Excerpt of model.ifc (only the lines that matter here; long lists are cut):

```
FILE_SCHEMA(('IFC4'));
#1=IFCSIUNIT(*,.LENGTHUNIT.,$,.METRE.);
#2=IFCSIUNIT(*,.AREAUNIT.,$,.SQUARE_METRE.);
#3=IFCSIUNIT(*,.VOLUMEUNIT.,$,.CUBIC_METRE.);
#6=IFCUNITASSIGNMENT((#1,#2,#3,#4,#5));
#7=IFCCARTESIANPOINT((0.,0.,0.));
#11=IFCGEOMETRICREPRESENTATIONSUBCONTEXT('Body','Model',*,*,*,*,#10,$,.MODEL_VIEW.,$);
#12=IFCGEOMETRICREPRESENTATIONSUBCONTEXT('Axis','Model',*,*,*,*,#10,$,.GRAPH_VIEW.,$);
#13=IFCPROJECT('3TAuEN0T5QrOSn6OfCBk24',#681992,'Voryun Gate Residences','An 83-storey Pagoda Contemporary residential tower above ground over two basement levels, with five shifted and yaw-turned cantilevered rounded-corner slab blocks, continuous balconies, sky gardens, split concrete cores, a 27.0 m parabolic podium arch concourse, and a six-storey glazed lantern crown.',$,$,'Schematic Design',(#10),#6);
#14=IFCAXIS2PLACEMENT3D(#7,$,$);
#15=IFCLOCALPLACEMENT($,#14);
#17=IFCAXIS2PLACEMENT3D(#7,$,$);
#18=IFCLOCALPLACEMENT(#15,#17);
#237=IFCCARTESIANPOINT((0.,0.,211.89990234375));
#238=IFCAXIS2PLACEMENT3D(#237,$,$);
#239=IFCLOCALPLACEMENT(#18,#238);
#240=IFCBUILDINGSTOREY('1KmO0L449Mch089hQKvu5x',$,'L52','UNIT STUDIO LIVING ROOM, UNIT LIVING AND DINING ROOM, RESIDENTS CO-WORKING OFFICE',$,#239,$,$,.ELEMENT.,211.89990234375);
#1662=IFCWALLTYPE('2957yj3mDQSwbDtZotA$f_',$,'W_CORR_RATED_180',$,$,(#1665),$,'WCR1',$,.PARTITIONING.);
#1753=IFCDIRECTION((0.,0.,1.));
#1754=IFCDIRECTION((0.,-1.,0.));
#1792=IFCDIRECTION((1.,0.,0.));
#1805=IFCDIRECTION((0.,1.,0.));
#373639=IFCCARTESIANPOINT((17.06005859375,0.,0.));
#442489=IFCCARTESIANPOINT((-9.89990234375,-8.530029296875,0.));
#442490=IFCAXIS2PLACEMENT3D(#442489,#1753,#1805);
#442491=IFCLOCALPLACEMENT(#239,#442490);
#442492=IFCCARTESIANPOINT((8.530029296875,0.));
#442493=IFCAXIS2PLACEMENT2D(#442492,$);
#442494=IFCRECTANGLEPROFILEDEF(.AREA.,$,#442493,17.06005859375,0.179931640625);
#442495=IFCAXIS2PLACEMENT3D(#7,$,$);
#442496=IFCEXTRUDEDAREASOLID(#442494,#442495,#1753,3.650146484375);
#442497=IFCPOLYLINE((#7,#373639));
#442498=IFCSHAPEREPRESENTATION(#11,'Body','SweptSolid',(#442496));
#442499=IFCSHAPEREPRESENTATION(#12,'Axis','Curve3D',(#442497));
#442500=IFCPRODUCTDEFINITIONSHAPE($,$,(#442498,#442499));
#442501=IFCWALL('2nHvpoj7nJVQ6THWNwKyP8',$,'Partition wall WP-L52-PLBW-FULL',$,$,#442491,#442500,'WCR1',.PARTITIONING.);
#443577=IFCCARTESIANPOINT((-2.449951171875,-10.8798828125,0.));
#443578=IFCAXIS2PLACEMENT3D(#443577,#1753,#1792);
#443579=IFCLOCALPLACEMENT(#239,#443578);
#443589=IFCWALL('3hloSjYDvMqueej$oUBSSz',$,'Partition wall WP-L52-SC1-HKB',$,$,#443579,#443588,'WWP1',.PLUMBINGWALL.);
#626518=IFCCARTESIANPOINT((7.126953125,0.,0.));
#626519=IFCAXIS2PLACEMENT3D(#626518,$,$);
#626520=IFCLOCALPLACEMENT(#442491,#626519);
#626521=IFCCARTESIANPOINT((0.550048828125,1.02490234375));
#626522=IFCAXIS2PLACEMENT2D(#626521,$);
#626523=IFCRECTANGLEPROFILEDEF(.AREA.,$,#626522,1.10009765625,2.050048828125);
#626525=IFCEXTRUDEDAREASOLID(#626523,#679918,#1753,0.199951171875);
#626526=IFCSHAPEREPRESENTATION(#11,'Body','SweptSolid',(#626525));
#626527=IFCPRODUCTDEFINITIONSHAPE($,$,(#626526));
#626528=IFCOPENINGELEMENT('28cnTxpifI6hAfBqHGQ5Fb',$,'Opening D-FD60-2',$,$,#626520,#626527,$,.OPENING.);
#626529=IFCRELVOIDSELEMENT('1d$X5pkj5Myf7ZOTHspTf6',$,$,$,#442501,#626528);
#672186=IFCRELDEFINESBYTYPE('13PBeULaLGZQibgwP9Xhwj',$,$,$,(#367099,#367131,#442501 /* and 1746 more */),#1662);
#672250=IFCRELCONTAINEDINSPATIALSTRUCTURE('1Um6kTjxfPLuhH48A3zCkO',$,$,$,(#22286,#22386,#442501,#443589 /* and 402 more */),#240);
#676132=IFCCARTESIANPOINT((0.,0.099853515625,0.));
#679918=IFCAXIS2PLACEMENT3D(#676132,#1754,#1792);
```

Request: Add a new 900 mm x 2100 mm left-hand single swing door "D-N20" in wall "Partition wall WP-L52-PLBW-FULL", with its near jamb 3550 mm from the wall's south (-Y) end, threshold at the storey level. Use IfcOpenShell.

```python
import numpy as np
import ifcopenshell
import ifcopenshell.api.feature
import ifcopenshell.api.geometry
import ifcopenshell.api.root
import ifcopenshell.api.spatial
import ifcopenshell.geom
import ifcopenshell.util.element
import ifcopenshell.util.placement
import ifcopenshell.util.representation
import ifcopenshell.util.shape
import ifcopenshell.util.unit

model = ifcopenshell.open("model.ifc")
unit_scale = ifcopenshell.util.unit.calculate_unit_scale(model)
settings = ifcopenshell.geom.settings()


def volume(element):
    """Net volume in cubic metres, openings subtracted."""
    shape = ifcopenshell.geom.create_shape(settings, element)
    return ifcopenshell.util.shape.get_volume(shape.geometry)


wall = model.by_id(442501)
storey = ifcopenshell.util.element.get_container(wall, ifc_class="IfcBuildingStorey")
context = ifcopenshell.util.representation.get_context(model, "Model", "Body", "MODEL_VIEW")
before = volume(wall)

width, height, from_end, sill = 0.9, 2.1, 3.55, 0.0  # metres

# The wall runs along its own X axis, and the end named is its -X end.
wall_shape = ifcopenshell.geom.create_shape(settings, wall)
x, y, z = ifcopenshell.util.shape.get_vertices(wall_shape.geometry).T
start = x.min() + from_end
face, thickness = float(y.min()), float(y.max() - y.min())
wall_matrix = ifcopenshell.util.placement.get_local_placement(wall.ObjectPlacement)
level = ifcopenshell.util.placement.get_local_placement(storey.ObjectPlacement)[2, 3]


def in_wall(x, y):
    """Placement at x, y metres in the wall's axes, at sill height."""
    matrix = wall_matrix.copy()
    matrix[:, 3] = wall_matrix @ np.array([x / unit_scale, y / unit_scale, 0.0, 1.0])
    matrix[2, 3] = level + sill / unit_scale
    return matrix


# Opening: a box that overshoots both wall faces by 50 mm.
opening = ifcopenshell.api.root.create_entity(model, ifc_class="IfcOpeningElement", predefined_type="OPENING")
box = ifcopenshell.api.geometry.add_wall_representation(
    model, context=context, length=width, height=height, thickness=thickness + 0.1
)
ifcopenshell.api.geometry.assign_representation(model, product=opening, representation=box)
ifcopenshell.api.geometry.edit_object_placement(model, product=opening, matrix=in_wall(start, face - 0.05), is_si=False)
ifcopenshell.api.feature.add_feature(model, feature=opening, element=wall)

door = ifcopenshell.api.root.create_entity(model, ifc_class="IfcDoor", name="D-N20", predefined_type="DOOR")
door.OverallWidth, door.OverallHeight = width / unit_scale, height / unit_scale
door.OperationType = "SINGLE_SWING_LEFT"
body = ifcopenshell.api.geometry.add_door_representation(
    model,
    context=context,
    overall_width=door.OverallWidth,
    overall_height=door.OverallHeight,
    operation_type="SINGLE_SWING_LEFT",
    lining_properties={"LiningDepth": thickness / unit_scale, "ThresholdDepth": thickness / unit_scale},
)
ifcopenshell.api.geometry.assign_representation(model, product=door, representation=body)
ifcopenshell.api.spatial.assign_container(model, products=[door], relating_structure=storey)
ifcopenshell.api.feature.add_filling(model, opening=opening, element=door)

# The lining spans the wall, so the door starts at the wall face.
ifcopenshell.api.geometry.edit_object_placement(model, product=door, matrix=in_wall(start, face), is_si=False)

after = volume(wall)

print(f"wall volume {before:.3f} -> {after:.3f} m3")

model.write("model_edited.ifc")
```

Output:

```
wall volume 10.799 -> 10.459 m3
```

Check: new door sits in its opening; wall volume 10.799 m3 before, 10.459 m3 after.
